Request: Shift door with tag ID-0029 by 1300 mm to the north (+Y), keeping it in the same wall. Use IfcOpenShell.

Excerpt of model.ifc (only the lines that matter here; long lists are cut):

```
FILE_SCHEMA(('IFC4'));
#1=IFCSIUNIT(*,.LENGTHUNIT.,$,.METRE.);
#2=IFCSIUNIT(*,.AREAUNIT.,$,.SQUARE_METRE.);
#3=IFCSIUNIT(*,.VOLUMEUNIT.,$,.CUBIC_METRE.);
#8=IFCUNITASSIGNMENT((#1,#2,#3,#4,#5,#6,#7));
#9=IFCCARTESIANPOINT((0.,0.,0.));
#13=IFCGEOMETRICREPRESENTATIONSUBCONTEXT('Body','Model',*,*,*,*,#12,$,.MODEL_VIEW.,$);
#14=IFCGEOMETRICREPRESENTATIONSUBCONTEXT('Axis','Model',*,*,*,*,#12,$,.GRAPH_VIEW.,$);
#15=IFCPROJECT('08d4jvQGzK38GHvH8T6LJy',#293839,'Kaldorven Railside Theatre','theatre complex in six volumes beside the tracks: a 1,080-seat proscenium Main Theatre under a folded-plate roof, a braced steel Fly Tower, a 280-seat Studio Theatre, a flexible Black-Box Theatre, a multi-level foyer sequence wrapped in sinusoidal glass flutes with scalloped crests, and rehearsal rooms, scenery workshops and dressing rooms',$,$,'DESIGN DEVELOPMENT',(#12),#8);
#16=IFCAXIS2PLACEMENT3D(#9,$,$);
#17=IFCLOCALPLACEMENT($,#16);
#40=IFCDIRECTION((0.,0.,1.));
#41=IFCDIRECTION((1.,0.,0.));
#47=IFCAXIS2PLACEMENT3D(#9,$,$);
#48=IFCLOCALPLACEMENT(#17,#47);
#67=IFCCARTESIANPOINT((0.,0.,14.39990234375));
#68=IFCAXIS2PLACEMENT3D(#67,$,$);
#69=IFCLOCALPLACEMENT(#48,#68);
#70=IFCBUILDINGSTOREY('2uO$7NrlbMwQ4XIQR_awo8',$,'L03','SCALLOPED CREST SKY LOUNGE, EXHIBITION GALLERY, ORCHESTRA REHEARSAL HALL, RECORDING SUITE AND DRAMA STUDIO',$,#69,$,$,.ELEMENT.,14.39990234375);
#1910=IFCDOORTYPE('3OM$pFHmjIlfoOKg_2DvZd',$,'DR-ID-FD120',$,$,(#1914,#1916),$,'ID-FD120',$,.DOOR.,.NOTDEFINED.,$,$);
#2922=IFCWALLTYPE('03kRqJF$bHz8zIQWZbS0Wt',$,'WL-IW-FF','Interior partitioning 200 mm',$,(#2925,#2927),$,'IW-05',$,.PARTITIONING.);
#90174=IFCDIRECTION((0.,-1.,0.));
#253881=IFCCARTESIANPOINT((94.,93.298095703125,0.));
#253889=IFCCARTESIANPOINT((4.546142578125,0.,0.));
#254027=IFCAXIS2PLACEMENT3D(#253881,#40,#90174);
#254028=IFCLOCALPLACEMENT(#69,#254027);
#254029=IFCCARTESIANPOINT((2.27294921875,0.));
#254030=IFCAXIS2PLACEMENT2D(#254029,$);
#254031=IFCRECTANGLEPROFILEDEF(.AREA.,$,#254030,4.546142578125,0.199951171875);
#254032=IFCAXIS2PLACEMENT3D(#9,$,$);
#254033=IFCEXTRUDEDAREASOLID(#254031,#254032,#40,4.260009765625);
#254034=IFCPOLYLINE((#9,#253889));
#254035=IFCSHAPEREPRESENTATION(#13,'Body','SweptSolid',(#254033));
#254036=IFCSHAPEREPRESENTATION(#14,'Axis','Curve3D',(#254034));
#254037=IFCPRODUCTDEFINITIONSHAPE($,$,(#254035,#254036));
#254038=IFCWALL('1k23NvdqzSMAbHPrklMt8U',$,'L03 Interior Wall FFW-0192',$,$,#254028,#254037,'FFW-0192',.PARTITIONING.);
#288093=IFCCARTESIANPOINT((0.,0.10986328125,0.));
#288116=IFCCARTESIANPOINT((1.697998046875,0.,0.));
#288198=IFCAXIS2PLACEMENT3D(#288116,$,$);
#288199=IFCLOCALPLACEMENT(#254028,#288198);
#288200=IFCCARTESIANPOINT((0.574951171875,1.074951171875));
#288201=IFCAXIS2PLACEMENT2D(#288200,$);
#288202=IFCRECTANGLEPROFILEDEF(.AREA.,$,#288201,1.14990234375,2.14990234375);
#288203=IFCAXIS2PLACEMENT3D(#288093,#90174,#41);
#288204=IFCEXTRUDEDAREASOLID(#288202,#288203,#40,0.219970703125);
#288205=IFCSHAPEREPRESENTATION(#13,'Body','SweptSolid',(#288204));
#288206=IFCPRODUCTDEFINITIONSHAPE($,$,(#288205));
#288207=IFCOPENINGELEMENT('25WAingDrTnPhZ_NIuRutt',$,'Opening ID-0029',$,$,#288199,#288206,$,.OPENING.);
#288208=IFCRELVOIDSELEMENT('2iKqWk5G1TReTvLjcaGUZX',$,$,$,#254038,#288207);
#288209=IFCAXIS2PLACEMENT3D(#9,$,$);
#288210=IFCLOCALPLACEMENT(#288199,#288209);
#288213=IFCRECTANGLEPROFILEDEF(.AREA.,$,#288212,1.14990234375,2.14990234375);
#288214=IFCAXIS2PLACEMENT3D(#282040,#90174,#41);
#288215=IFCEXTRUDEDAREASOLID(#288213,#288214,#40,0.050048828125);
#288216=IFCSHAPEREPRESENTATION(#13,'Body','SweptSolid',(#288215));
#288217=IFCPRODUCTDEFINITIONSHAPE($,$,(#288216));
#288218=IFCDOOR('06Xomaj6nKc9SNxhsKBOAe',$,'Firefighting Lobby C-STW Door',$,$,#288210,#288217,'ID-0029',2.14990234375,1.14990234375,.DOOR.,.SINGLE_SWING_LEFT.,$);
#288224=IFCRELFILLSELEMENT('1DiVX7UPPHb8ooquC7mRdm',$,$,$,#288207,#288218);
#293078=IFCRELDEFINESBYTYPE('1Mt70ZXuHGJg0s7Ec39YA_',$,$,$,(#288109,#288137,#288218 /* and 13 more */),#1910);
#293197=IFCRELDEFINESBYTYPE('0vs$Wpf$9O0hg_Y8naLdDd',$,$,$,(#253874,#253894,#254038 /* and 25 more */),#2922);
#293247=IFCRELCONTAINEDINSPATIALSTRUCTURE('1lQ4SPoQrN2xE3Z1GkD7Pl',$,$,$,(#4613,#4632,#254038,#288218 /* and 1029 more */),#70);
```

```python
import ifcopenshell
import ifcopenshell.api.geometry
import ifcopenshell.util.placement

model = ifcopenshell.open("model.ifc")

door = model.by_guid("06Xomaj6nKc9SNxhsKBOAe")
opening = door.FillsVoids[0].RelatingOpeningElement
wall = opening.VoidsElements[0].RelatingBuildingElement

wall_matrix = ifcopenshell.util.placement.get_local_placement(wall.ObjectPlacement)
shift = wall_matrix[:3, 0] * -1.3
before = ifcopenshell.util.placement.get_local_placement(door.ObjectPlacement)[:3, 3].copy()

# The door is placed relative to its opening, so it follows when the opening moves.
matrix = ifcopenshell.util.placement.get_local_placement(opening.ObjectPlacement)
matrix[:3, 3] += shift
ifcopenshell.api.geometry.edit_object_placement(
    model, product=opening, matrix=matrix, is_si=False, should_transform_children=True
)

after = ifcopenshell.util.placement.get_local_placement(door.ObjectPlacement)[:3, 3]
print("door moved by", (after - before).round(3) + 0.0)

model.write("model_rev.ifc")
```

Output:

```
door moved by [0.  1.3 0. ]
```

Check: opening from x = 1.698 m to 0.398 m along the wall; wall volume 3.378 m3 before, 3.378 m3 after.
